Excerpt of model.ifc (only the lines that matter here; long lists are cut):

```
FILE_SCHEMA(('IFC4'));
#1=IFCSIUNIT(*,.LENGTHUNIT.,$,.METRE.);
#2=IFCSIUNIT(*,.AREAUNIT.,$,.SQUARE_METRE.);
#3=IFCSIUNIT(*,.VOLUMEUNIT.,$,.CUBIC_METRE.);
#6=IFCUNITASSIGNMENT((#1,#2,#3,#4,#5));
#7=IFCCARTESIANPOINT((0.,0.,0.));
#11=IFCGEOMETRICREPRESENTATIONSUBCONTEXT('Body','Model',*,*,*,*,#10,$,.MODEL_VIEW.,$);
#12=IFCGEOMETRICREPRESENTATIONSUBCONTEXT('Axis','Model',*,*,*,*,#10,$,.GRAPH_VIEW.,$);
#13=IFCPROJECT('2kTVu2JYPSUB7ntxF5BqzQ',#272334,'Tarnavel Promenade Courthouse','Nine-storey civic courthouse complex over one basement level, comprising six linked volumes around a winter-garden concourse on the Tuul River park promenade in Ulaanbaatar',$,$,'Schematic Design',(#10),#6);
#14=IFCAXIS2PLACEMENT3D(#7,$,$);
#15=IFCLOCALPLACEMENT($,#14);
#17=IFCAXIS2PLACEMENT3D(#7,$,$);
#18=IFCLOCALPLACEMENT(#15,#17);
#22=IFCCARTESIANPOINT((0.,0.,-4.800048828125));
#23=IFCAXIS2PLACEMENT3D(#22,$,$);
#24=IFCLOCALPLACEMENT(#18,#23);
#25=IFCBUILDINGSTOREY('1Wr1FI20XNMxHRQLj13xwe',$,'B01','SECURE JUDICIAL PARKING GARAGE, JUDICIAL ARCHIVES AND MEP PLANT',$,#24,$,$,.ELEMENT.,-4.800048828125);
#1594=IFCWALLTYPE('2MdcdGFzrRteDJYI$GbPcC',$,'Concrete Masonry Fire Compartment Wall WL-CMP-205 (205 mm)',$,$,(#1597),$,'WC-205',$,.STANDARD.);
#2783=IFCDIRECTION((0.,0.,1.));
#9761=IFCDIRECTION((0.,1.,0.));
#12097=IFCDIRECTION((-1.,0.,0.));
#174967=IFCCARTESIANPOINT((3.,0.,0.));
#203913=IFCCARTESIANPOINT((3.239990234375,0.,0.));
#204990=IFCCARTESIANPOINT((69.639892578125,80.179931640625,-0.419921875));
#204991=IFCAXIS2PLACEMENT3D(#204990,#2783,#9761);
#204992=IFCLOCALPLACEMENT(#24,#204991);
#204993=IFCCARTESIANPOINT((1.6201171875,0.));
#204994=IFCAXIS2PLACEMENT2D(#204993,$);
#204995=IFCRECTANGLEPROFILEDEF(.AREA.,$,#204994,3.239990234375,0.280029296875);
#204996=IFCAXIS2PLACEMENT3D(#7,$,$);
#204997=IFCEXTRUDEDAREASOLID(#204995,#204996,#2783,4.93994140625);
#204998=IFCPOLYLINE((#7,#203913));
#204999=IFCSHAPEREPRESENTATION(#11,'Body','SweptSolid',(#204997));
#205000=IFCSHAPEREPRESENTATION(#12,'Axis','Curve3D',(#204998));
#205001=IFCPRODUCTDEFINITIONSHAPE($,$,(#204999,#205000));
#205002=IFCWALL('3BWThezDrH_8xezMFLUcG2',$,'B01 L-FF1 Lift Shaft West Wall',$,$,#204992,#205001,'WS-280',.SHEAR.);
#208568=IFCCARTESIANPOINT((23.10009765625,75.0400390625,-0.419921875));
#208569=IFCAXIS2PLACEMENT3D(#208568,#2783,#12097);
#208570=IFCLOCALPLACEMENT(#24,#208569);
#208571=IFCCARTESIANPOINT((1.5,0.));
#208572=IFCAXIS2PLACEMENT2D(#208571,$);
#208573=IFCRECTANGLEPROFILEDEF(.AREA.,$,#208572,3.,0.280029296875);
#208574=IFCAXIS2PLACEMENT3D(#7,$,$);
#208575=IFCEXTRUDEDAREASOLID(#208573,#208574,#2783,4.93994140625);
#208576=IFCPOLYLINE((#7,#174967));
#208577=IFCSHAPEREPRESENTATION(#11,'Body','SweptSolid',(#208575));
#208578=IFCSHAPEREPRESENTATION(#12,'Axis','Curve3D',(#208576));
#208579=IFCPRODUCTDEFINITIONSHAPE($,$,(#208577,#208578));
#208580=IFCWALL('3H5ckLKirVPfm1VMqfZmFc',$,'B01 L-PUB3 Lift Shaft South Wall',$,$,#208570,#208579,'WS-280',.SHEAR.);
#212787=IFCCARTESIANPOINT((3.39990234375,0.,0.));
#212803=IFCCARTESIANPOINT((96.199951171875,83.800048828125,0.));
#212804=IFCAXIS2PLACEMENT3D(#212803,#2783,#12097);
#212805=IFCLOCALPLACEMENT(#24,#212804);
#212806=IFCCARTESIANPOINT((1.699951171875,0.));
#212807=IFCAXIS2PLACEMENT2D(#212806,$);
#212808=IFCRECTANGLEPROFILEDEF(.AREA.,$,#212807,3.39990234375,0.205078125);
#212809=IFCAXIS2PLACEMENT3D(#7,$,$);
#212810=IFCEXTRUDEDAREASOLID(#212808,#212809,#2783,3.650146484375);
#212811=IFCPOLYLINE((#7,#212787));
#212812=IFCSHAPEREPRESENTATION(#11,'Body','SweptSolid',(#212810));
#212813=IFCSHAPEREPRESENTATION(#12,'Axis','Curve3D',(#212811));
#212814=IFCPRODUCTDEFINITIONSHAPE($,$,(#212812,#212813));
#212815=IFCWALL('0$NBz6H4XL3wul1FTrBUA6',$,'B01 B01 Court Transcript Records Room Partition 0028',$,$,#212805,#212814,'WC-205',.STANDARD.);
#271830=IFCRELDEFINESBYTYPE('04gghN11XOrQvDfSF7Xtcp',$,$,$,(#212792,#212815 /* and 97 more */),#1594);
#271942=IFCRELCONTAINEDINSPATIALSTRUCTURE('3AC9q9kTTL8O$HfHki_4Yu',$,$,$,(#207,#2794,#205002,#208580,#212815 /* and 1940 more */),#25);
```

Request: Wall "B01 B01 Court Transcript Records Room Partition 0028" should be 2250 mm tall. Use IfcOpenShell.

```python
import ifcopenshell
import ifcopenshell.geom
import ifcopenshell.util.representation
import ifcopenshell.util.shape
import ifcopenshell.util.unit

model = ifcopenshell.open("model.ifc")
unit_scale = ifcopenshell.util.unit.calculate_unit_scale(model)
settings = ifcopenshell.geom.settings()


def volume(element):
    """Net volume in cubic metres, openings subtracted."""
    shape = ifcopenshell.geom.create_shape(settings, element)
    return ifcopenshell.util.shape.get_volume(shape.geometry)


wall = model.by_guid("0$NBz6H4XL3wul1FTrBUA6")
before = volume(wall)

body = ifcopenshell.util.representation.get_representation(wall, "Model", "Body")
solid = body.Items[0]
old_height = solid.Depth
solid.Depth = 2.25 / unit_scale
after = volume(wall)

print(f"height {old_height:g} -> {solid.Depth:g}, volume {before:.3f} -> {after:.3f} m3")

model.write("model_v2.ifc")
```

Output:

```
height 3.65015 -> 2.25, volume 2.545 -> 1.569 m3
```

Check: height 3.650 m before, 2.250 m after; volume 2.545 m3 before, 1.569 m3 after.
